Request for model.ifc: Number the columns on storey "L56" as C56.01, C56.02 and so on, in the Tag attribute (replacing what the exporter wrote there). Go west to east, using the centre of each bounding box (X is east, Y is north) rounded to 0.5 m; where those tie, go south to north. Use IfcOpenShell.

First a look at what the model holds.

```python
import ifcopenshell
import ifcopenshell.util.element
import ifcopenshell.util.placement

model = ifcopenshell.open("model.ifc")
print(model.schema)
storey = next(s for s in model.by_type("IfcBuildingStorey") if s.Name == "L56")
columns = [e for e in ifcopenshell.util.element.get_decomposition(storey) if e.is_a("IfcColumn")]
for e in sorted(columns, key=lambda e: e.id()):
    origin = ifcopenshell.util.placement.get_local_placement(e.ObjectPlacement)[:3, 3]
    print(e.id(), e.Tag, e.Name, origin.round(2) + 0.0, sep=" | ")
```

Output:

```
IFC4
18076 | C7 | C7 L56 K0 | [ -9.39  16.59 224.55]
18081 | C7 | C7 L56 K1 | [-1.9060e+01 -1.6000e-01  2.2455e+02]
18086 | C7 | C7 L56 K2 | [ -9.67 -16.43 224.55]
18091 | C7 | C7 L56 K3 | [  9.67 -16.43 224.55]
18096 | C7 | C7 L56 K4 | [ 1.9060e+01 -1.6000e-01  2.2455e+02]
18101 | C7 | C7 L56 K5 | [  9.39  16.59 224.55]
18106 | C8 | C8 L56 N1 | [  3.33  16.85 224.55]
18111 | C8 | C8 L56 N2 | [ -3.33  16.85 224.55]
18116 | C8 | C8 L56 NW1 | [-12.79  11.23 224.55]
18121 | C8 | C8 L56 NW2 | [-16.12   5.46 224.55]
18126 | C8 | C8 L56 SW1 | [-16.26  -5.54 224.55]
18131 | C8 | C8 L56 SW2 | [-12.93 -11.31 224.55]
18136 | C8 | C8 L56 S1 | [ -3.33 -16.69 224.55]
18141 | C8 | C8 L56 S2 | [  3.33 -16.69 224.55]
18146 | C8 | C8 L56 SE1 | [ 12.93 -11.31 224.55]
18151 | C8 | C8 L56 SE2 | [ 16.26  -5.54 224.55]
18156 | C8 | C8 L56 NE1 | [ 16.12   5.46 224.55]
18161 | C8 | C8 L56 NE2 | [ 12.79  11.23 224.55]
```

```python
import ifcopenshell
import ifcopenshell.geom
import ifcopenshell.util.element
import ifcopenshell.util.shape

model = ifcopenshell.open("model.ifc")
settings = ifcopenshell.geom.settings()
settings.set("use-world-coords", True)


def centre(element):
    shape = ifcopenshell.geom.create_shape(settings, element)
    return ifcopenshell.util.shape.get_bbox_centroid(shape.geometry)


storey = next(s for s in model.by_type("IfcBuildingStorey") if s.Name == "L56")
columns = [e for e in ifcopenshell.util.element.get_decomposition(storey) if e.is_a("IfcColumn")]

# Insertion points can sit at a corner or the storey origin, so sort by the geometry (in metres).
centres = {e: centre(e) for e in columns}
columns.sort(key=lambda e: (round(centres[e][0] / 0.5), centres[e][1]))

for i, e in enumerate(columns, start=1):
    number = f"C56.{i:02d}"
    e.Tag = number
    print(e.id(), number)

model.write("model_edited.ifc")
```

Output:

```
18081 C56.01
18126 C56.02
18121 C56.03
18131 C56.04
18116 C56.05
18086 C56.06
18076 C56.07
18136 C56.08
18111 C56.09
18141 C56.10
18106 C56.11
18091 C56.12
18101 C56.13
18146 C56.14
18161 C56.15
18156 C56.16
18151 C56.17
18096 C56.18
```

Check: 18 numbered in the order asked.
